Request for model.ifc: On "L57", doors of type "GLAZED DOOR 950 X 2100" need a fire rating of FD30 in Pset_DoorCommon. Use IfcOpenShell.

First a look at what the model holds.

```python
import ifcopenshell
import ifcopenshell.util.element

model = ifcopenshell.open("model.ifc")
print(model.schema)
storey = next(s for s in model.by_type("IfcBuildingStorey") if s.Name == "L57")
doors = [e for e in ifcopenshell.util.element.get_decomposition(storey) if e.is_a("IfcDoor")]
seen = {}
for e in doors:
    element_type = ifcopenshell.util.element.get_type(e)
    key = (element_type.Name if element_type != e and element_type else None, ifcopenshell.util.element.get_pset(e, "Pset_DoorCommon", "FireRating"))
    seen[key] = seen.get(key, 0) + 1
for (name, value), count in sorted(seen.items(), key=str):
    print(count, "x", name, "|", value)
```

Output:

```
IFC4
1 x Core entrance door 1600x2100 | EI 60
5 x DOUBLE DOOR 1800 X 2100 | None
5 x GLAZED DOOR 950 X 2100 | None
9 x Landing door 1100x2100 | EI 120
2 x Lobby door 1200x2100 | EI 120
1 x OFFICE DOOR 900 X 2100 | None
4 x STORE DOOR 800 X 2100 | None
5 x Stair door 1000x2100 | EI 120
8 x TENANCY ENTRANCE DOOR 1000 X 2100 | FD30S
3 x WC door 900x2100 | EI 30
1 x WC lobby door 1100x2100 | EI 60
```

```python
import ifcopenshell
import ifcopenshell.api.pset
import ifcopenshell.util.element

model = ifcopenshell.open("model.ifc")

storey = next(s for s in model.by_type("IfcBuildingStorey") if s.Name == "L57")
doors = [e for e in ifcopenshell.util.element.get_decomposition(storey) if e.is_a("IfcDoor")]

count = 0
for e in doors:
    element_type = ifcopenshell.util.element.get_type(e)
    if element_type in (None, e) or element_type.Name != "GLAZED DOOR 950 X 2100":
        continue
    found = ifcopenshell.util.element.get_pset(e, "Pset_DoorCommon", should_inherit=False)
    if found:
        pset = model.by_id(found["id"])
        if len(ifcopenshell.util.element.get_elements_by_pset(pset)) > 1:
            pset = ifcopenshell.api.pset.unshare_pset(model, products=[e], pset=pset)[0]
    else:
        pset = ifcopenshell.api.pset.add_pset(model, product=e, name="Pset_DoorCommon")
    ifcopenshell.api.pset.edit_pset(model, pset=pset, properties={"FireRating": "FD30"})
    count += 1

print(count, "doors updated")

model.write("model_updated.ifc")
```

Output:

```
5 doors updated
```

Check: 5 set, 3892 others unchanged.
